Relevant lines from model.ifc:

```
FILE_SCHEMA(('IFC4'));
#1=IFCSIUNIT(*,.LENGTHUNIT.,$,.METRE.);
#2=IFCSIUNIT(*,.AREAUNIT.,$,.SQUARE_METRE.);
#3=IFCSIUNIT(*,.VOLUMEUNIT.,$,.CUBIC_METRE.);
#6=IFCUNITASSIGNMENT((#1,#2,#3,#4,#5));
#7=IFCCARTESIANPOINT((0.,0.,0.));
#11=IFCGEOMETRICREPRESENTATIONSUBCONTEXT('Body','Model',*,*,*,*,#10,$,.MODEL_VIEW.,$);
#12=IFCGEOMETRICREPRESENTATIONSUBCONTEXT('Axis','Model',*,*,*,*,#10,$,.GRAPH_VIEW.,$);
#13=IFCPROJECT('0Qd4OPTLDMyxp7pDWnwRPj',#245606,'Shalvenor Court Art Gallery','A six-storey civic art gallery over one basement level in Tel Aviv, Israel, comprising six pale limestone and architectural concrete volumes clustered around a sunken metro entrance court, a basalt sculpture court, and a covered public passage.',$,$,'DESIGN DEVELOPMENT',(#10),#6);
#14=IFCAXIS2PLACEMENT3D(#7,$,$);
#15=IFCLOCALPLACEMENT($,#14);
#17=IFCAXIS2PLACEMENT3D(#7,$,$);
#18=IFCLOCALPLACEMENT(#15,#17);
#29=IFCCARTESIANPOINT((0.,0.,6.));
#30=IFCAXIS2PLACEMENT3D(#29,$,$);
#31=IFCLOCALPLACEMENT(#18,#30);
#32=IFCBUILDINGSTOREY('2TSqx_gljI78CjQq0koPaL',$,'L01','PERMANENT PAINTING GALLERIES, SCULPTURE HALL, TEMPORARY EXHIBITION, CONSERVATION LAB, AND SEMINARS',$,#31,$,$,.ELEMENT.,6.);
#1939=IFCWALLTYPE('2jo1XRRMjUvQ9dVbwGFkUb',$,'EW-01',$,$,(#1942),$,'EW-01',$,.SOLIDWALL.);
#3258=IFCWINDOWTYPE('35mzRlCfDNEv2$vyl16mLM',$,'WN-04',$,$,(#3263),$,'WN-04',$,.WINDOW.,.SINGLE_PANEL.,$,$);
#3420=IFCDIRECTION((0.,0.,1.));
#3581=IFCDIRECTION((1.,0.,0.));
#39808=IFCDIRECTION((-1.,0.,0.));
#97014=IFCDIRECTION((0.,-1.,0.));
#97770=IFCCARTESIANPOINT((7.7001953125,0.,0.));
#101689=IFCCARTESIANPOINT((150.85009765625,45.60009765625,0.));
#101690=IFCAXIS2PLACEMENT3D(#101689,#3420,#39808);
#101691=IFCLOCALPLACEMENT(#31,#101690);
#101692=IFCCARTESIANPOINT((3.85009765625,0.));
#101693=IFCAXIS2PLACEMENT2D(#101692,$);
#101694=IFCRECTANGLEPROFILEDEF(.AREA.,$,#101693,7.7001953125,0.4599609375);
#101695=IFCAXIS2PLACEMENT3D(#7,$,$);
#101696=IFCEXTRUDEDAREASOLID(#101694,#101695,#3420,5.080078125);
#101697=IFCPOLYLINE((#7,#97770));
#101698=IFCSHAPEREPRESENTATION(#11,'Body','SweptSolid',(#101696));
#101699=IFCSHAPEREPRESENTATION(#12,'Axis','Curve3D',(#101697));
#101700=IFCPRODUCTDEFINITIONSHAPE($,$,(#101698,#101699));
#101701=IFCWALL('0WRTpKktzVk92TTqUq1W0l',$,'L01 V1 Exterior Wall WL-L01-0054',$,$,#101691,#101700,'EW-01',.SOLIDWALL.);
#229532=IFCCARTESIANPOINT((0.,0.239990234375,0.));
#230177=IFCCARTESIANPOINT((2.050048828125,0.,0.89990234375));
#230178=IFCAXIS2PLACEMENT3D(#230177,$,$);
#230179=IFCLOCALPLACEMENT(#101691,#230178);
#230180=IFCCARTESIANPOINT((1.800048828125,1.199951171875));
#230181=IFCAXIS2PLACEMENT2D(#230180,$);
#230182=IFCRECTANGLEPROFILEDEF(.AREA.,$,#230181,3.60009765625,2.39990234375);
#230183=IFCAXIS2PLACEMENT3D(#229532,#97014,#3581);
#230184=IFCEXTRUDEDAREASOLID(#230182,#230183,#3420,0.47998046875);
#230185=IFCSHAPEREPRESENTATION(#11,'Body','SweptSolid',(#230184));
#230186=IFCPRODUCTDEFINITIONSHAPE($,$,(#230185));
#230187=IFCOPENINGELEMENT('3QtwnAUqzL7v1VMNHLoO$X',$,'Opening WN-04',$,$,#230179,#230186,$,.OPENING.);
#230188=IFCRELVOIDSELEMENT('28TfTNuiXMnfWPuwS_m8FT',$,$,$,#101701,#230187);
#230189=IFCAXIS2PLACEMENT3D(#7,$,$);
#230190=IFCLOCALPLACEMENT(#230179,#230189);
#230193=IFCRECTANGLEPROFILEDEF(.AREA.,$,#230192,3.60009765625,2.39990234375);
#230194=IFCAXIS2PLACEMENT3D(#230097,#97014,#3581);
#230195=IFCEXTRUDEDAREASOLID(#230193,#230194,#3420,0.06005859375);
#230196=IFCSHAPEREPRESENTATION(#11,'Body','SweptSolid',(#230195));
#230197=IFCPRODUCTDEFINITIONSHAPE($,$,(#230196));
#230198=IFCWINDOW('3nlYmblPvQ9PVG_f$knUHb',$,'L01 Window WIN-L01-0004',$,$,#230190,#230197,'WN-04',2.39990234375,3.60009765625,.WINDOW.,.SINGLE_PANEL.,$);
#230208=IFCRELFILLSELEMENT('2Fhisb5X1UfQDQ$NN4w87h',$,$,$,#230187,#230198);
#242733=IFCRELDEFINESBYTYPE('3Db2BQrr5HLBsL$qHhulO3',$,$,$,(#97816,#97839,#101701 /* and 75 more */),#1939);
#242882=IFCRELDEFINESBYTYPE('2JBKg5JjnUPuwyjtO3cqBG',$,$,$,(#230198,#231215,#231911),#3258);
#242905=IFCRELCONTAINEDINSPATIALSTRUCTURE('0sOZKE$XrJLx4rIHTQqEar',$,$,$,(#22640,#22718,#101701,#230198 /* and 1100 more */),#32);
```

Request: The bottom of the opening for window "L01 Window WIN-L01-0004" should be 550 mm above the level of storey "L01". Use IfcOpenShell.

```python
import numpy as np
import ifcopenshell
import ifcopenshell.api.geometry
import ifcopenshell.geom
import ifcopenshell.util.element
import ifcopenshell.util.placement
import ifcopenshell.util.shape
import ifcopenshell.util.unit

model = ifcopenshell.open("model.ifc")
unit_scale = ifcopenshell.util.unit.calculate_unit_scale(model)

window = model.by_id(230198)
opening = window.FillsVoids[0].RelatingOpeningElement
storey = ifcopenshell.util.element.get_container(window, ifc_class="IfcBuildingStorey")
level = ifcopenshell.util.placement.get_local_placement(storey.ObjectPlacement)[2, 3]

# The opening's origin need not be at the sill, so measure its lowest point.
shape = ifcopenshell.geom.create_shape(ifcopenshell.geom.settings(), opening)
bottom = ifcopenshell.util.shape.get_shape_bottom_elevation(shape, shape.geometry) / unit_scale
dz = level + 0.55 / unit_scale - bottom

shift = np.array([0.0, 0.0, dz])
# The window is placed relative to its opening, so it follows when the opening moves.
matrix = ifcopenshell.util.placement.get_local_placement(opening.ObjectPlacement)
matrix[:3, 3] += shift
ifcopenshell.api.geometry.edit_object_placement(
    model, product=opening, matrix=matrix, is_si=False, should_transform_children=True
)

print(f"moved by {dz * unit_scale:+.3f} m")

model.write("model-out.ifc")
```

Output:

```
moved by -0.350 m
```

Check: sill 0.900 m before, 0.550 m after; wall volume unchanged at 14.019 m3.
